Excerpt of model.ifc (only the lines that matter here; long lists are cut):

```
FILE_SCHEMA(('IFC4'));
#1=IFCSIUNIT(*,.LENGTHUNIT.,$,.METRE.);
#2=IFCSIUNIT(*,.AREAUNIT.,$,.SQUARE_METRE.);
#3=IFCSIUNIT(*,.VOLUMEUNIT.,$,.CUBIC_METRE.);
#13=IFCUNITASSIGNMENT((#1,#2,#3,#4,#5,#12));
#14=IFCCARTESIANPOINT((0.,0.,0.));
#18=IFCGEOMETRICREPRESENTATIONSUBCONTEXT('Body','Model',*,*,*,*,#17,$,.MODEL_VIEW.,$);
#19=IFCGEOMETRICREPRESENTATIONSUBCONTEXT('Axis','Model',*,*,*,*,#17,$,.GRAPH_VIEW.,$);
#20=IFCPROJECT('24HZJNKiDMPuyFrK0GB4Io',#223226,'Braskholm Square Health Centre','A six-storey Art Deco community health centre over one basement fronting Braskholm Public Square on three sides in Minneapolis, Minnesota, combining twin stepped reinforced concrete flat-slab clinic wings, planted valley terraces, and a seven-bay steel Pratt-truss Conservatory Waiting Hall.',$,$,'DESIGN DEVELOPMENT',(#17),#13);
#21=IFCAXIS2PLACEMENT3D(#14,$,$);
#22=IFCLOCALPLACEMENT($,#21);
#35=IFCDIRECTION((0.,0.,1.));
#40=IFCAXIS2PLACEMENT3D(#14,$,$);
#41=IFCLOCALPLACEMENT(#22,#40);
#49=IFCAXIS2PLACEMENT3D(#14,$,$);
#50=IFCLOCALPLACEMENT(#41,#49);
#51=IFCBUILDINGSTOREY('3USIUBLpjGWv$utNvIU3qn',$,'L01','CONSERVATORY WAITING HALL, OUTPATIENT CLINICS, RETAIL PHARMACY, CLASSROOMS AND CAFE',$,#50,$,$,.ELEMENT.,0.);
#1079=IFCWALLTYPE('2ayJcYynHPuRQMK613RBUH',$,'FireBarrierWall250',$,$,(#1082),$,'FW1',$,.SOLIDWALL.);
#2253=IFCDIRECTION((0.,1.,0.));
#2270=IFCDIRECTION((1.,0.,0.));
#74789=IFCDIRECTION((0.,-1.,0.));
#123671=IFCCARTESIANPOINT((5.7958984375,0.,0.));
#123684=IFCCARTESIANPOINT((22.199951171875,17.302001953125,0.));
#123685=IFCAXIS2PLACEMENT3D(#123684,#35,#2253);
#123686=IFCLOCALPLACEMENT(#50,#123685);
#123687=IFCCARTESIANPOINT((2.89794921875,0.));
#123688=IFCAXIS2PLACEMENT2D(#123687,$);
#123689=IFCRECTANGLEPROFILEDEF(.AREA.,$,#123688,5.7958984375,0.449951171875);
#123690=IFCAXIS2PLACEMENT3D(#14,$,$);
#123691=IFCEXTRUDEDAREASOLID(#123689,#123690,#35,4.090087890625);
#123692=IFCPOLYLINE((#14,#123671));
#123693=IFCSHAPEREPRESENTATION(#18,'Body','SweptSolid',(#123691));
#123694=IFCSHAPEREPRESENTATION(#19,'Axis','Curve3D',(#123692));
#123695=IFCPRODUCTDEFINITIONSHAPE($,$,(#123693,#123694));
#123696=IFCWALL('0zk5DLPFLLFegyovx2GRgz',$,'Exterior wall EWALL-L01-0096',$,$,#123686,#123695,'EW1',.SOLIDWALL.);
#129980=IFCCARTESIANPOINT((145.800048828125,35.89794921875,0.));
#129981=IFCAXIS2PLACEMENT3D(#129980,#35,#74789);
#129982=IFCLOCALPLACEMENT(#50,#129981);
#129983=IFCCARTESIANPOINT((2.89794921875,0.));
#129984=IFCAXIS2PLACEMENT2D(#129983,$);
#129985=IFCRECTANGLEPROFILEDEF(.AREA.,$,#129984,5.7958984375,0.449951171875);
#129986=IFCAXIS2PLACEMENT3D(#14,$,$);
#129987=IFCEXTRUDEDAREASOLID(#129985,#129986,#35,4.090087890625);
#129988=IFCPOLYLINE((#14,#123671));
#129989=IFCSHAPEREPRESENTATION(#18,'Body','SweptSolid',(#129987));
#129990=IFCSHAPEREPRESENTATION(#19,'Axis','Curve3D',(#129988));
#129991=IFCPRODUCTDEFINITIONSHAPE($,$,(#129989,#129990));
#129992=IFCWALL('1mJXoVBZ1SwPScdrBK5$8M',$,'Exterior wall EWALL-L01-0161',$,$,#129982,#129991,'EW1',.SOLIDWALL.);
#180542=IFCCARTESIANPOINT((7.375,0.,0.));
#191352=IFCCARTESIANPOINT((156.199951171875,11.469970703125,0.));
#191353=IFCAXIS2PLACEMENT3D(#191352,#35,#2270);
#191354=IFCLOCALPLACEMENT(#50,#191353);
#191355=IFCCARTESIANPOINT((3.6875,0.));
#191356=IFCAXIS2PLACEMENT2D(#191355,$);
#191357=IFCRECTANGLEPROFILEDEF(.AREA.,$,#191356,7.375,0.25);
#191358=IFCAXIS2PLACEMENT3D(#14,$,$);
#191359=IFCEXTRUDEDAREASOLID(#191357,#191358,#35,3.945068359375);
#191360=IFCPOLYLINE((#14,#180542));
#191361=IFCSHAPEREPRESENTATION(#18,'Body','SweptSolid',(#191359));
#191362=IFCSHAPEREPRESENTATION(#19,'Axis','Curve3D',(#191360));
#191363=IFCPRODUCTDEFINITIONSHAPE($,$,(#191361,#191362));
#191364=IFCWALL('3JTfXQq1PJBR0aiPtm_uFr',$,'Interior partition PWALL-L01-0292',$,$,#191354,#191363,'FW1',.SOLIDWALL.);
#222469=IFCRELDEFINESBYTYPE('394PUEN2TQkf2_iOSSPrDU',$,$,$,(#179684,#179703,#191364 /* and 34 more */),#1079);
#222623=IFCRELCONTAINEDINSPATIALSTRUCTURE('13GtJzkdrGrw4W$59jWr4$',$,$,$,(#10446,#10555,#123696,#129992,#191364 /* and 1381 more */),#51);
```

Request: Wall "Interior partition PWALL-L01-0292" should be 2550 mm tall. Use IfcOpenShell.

```python
import ifcopenshell
import ifcopenshell.geom
import ifcopenshell.util.representation
import ifcopenshell.util.shape

model = ifcopenshell.open("model.ifc")
settings = ifcopenshell.geom.settings()


def volume(element):
    """Net volume in cubic metres, openings subtracted."""
    shape = ifcopenshell.geom.create_shape(settings, element)
    return ifcopenshell.util.shape.get_volume(shape.geometry)


wall = model.by_id(191364)
before = volume(wall)

body = ifcopenshell.util.representation.get_representation(wall, "Model", "Body")
solid = body.Items[0]
old_height = solid.Depth
solid.Depth = 2.55
after = volume(wall)

print(f"height {old_height:g} -> {solid.Depth:g}, volume {before:.3f} -> {after:.3f} m3")

model.write("model_v2.ifc")
```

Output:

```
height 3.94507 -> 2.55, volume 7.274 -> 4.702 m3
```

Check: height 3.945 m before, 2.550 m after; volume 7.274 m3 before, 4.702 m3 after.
